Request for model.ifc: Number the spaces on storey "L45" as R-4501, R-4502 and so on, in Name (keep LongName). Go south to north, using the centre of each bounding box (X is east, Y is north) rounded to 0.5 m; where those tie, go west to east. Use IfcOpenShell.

First a look at what the model holds.

```python
import ifcopenshell
import ifcopenshell.util.element
import ifcopenshell.util.placement

model = ifcopenshell.open("model.ifc")
print(model.schema)
storey = next(s for s in model.by_type("IfcBuildingStorey") if s.Name == "L45")
spaces = [e for e in ifcopenshell.util.element.get_decomposition(storey) if e.is_a("IfcSpace")]
for e in sorted(spaces, key=lambda e: e.id()):
    origin = ifcopenshell.util.placement.get_local_placement(e.ObjectPlacement)[:3, 3]
    print(e.id(), e.Name, e.LongName, origin.round(2) + 0.0, sep=" | ")
```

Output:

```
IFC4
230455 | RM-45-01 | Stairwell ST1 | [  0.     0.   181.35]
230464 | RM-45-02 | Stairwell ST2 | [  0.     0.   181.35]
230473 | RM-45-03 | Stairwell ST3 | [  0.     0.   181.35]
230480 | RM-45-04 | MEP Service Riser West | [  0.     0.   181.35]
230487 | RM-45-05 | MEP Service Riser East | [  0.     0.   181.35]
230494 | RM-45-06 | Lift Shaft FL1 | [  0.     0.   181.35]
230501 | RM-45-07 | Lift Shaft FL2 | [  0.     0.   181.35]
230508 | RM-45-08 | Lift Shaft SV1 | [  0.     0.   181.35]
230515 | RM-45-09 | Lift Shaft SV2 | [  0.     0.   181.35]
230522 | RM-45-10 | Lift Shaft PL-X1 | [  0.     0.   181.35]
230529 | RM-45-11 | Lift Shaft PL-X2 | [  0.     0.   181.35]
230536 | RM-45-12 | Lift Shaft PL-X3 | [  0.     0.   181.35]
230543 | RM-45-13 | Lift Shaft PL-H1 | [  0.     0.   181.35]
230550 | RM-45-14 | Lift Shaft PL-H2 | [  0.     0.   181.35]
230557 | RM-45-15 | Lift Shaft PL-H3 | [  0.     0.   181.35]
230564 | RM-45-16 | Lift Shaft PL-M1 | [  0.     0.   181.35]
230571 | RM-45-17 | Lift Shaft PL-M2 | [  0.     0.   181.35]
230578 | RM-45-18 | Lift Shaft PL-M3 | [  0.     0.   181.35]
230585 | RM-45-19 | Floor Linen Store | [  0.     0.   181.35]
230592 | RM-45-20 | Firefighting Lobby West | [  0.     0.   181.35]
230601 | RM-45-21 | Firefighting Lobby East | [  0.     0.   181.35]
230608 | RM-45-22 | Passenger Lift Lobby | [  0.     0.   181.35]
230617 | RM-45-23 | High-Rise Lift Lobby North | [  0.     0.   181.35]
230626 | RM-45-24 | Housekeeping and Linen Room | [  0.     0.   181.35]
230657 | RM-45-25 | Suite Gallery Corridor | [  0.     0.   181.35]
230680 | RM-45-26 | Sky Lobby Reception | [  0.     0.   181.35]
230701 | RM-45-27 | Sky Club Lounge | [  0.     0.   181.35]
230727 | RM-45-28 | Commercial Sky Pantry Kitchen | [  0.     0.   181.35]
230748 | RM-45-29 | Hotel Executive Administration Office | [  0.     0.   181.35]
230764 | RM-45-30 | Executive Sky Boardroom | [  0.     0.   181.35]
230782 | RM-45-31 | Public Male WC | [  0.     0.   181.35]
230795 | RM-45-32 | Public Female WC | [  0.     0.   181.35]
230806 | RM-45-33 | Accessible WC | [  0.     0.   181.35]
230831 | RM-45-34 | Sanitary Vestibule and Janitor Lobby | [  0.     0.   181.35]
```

```python
import ifcopenshell
import ifcopenshell.geom
import ifcopenshell.util.element
import ifcopenshell.util.shape

model = ifcopenshell.open("model.ifc")
settings = ifcopenshell.geom.settings()
settings.set("use-world-coords", True)


def centre(element):
    shape = ifcopenshell.geom.create_shape(settings, element)
    return ifcopenshell.util.shape.get_bbox_centroid(shape.geometry)


storey = next(s for s in model.by_type("IfcBuildingStorey") if s.Name == "L45")
spaces = [e for e in ifcopenshell.util.element.get_decomposition(storey) if e.is_a("IfcSpace")]

# Insertion points can sit at a corner or the storey origin, so sort by the geometry (in metres).
centres = {e: centre(e) for e in spaces}
spaces.sort(key=lambda e: (round(centres[e][1] / 0.5), centres[e][0]))

for i, e in enumerate(spaces, start=1):
    number = f"R-45{i:02d}"
    e.Name = number
    print(e.id(), number)

model.write("model_v2.ifc")
```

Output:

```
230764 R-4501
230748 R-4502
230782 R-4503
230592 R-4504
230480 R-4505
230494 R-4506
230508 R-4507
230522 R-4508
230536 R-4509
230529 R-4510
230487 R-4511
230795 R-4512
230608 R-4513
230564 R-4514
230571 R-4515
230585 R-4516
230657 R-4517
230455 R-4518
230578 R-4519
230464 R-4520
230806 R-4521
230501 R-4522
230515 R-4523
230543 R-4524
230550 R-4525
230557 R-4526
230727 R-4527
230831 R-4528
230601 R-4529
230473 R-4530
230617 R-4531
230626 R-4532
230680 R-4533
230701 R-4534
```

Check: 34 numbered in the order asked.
